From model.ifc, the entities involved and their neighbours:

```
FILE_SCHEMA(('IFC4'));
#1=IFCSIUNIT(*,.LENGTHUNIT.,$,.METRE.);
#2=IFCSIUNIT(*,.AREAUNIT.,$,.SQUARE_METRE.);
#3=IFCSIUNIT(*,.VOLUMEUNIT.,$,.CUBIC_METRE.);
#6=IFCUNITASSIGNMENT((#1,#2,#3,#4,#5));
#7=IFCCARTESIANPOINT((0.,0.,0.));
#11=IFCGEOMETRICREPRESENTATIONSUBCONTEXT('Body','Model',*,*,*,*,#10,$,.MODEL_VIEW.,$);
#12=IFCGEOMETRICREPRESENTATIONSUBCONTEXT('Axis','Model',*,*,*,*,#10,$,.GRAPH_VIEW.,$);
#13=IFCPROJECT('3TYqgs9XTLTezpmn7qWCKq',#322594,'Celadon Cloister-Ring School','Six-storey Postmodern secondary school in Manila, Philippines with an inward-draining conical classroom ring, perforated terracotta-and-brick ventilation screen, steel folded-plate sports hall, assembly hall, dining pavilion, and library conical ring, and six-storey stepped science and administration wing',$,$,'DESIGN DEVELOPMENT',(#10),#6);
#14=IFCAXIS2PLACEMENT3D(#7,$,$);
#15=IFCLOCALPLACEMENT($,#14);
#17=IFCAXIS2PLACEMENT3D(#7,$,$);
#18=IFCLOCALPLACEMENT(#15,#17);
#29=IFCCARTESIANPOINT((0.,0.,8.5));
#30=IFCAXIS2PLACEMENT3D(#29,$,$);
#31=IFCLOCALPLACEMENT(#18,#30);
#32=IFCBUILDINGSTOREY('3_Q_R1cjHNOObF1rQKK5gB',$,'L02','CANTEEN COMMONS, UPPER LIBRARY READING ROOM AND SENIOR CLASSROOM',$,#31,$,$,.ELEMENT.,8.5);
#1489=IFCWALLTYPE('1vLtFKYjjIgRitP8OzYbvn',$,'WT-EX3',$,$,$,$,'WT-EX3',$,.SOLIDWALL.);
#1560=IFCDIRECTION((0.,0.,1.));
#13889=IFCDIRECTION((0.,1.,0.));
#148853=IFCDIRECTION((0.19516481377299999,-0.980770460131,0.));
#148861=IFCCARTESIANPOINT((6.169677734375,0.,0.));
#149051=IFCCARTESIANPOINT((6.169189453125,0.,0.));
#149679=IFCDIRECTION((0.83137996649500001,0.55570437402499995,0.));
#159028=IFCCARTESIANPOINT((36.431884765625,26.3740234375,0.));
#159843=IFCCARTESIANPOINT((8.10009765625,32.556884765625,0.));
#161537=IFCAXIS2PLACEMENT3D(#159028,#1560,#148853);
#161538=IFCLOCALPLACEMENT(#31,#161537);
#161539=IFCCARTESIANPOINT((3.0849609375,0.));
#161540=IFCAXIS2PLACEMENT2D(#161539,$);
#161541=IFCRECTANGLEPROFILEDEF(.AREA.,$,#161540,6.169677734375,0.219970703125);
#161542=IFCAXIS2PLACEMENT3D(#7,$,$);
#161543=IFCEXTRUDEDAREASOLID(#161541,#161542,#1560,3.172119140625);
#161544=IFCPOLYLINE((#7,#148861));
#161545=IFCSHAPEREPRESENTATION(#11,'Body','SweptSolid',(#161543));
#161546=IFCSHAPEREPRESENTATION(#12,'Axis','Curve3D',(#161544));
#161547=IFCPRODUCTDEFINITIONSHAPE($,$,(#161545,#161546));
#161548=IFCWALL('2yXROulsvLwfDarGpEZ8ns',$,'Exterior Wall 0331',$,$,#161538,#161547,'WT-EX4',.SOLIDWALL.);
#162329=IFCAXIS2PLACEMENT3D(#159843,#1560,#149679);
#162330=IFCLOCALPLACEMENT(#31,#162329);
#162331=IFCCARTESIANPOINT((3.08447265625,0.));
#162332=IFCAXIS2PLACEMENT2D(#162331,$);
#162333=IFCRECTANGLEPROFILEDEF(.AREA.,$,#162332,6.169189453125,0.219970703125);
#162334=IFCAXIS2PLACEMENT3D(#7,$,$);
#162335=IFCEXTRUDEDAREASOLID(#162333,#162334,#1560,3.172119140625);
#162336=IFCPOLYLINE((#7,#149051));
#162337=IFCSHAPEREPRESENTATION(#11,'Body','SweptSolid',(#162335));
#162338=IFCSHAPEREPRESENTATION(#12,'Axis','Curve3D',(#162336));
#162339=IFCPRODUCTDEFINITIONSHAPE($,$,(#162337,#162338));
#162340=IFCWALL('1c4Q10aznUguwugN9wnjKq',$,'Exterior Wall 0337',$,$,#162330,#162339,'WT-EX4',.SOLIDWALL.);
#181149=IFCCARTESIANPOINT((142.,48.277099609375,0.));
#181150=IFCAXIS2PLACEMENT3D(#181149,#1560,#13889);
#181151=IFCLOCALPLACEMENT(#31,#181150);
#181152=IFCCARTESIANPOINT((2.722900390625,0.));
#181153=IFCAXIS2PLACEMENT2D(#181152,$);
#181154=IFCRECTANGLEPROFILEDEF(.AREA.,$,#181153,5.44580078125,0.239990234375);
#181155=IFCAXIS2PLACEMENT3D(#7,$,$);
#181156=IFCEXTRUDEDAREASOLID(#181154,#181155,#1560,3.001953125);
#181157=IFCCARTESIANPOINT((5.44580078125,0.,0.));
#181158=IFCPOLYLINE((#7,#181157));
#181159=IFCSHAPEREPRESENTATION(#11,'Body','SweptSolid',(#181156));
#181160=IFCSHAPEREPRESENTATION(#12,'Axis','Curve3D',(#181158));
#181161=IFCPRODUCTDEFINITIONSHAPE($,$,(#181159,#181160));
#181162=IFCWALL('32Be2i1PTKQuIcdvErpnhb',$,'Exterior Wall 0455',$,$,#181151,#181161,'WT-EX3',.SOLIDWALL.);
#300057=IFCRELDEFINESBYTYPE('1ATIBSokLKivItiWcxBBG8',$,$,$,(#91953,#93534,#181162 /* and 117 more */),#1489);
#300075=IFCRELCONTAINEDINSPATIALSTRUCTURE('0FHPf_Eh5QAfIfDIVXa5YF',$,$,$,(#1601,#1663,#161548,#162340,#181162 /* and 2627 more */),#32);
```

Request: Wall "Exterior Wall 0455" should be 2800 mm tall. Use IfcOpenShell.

```python
import ifcopenshell
import ifcopenshell.geom
import ifcopenshell.util.representation
import ifcopenshell.util.shape
import ifcopenshell.util.unit

model = ifcopenshell.open("model.ifc")
unit_scale = ifcopenshell.util.unit.calculate_unit_scale(model)
settings = ifcopenshell.geom.settings()


def volume(element):
    """Net volume in cubic metres, openings subtracted."""
    shape = ifcopenshell.geom.create_shape(settings, element)
    return ifcopenshell.util.shape.get_volume(shape.geometry)


wall = model.by_id(181162)
before = volume(wall)

body = ifcopenshell.util.representation.get_representation(wall, "Model", "Body")
solid = body.Items[0]
old_height = solid.Depth
solid.Depth = 2.8 / unit_scale
after = volume(wall)

print(f"height {old_height:g} -> {solid.Depth:g}, volume {before:.3f} -> {after:.3f} m3")

model.write("model-out.ifc")
```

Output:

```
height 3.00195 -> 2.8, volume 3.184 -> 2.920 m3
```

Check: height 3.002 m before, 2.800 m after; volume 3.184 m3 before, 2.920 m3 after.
